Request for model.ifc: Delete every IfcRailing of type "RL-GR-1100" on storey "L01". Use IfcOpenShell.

First a look at what the model holds.

```python
import ifcopenshell
import ifcopenshell.util.element

model = ifcopenshell.open("model.ifc")
print(model.schema)
storey = next(s for s in model.by_type("IfcBuildingStorey") if s.Name == "L01")
railings = [e for e in ifcopenshell.util.element.get_decomposition(storey) if e.is_a("IfcRailing")]
seen = {}
for e in railings:
    element_type = ifcopenshell.util.element.get_type(e)
    name = element_type.Name if element_type not in (None, e) else None
    seen[name] = seen.get(name, 0) + 1
for name, count in sorted(seen.items(), key=str):
    print(count, "x", name)
```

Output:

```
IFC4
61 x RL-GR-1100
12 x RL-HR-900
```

```python
import ifcopenshell
import ifcopenshell.api.root
import ifcopenshell.util.element

model = ifcopenshell.open("model.ifc")

storey = next(s for s in model.by_type("IfcBuildingStorey") if s.Name == "L01")
railings = [e for e in ifcopenshell.util.element.get_decomposition(storey) if e.is_a("IfcRailing")]
targets = [e for e in railings if (t := ifcopenshell.util.element.get_type(e)) not in (None, e) and t.Name == "RL-GR-1100"]

for e in targets:
    ifcopenshell.api.root.remove_product(model, product=e)
print(len(targets), "removed")

model.write("model_rev.ifc")
```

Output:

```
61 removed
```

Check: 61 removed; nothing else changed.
